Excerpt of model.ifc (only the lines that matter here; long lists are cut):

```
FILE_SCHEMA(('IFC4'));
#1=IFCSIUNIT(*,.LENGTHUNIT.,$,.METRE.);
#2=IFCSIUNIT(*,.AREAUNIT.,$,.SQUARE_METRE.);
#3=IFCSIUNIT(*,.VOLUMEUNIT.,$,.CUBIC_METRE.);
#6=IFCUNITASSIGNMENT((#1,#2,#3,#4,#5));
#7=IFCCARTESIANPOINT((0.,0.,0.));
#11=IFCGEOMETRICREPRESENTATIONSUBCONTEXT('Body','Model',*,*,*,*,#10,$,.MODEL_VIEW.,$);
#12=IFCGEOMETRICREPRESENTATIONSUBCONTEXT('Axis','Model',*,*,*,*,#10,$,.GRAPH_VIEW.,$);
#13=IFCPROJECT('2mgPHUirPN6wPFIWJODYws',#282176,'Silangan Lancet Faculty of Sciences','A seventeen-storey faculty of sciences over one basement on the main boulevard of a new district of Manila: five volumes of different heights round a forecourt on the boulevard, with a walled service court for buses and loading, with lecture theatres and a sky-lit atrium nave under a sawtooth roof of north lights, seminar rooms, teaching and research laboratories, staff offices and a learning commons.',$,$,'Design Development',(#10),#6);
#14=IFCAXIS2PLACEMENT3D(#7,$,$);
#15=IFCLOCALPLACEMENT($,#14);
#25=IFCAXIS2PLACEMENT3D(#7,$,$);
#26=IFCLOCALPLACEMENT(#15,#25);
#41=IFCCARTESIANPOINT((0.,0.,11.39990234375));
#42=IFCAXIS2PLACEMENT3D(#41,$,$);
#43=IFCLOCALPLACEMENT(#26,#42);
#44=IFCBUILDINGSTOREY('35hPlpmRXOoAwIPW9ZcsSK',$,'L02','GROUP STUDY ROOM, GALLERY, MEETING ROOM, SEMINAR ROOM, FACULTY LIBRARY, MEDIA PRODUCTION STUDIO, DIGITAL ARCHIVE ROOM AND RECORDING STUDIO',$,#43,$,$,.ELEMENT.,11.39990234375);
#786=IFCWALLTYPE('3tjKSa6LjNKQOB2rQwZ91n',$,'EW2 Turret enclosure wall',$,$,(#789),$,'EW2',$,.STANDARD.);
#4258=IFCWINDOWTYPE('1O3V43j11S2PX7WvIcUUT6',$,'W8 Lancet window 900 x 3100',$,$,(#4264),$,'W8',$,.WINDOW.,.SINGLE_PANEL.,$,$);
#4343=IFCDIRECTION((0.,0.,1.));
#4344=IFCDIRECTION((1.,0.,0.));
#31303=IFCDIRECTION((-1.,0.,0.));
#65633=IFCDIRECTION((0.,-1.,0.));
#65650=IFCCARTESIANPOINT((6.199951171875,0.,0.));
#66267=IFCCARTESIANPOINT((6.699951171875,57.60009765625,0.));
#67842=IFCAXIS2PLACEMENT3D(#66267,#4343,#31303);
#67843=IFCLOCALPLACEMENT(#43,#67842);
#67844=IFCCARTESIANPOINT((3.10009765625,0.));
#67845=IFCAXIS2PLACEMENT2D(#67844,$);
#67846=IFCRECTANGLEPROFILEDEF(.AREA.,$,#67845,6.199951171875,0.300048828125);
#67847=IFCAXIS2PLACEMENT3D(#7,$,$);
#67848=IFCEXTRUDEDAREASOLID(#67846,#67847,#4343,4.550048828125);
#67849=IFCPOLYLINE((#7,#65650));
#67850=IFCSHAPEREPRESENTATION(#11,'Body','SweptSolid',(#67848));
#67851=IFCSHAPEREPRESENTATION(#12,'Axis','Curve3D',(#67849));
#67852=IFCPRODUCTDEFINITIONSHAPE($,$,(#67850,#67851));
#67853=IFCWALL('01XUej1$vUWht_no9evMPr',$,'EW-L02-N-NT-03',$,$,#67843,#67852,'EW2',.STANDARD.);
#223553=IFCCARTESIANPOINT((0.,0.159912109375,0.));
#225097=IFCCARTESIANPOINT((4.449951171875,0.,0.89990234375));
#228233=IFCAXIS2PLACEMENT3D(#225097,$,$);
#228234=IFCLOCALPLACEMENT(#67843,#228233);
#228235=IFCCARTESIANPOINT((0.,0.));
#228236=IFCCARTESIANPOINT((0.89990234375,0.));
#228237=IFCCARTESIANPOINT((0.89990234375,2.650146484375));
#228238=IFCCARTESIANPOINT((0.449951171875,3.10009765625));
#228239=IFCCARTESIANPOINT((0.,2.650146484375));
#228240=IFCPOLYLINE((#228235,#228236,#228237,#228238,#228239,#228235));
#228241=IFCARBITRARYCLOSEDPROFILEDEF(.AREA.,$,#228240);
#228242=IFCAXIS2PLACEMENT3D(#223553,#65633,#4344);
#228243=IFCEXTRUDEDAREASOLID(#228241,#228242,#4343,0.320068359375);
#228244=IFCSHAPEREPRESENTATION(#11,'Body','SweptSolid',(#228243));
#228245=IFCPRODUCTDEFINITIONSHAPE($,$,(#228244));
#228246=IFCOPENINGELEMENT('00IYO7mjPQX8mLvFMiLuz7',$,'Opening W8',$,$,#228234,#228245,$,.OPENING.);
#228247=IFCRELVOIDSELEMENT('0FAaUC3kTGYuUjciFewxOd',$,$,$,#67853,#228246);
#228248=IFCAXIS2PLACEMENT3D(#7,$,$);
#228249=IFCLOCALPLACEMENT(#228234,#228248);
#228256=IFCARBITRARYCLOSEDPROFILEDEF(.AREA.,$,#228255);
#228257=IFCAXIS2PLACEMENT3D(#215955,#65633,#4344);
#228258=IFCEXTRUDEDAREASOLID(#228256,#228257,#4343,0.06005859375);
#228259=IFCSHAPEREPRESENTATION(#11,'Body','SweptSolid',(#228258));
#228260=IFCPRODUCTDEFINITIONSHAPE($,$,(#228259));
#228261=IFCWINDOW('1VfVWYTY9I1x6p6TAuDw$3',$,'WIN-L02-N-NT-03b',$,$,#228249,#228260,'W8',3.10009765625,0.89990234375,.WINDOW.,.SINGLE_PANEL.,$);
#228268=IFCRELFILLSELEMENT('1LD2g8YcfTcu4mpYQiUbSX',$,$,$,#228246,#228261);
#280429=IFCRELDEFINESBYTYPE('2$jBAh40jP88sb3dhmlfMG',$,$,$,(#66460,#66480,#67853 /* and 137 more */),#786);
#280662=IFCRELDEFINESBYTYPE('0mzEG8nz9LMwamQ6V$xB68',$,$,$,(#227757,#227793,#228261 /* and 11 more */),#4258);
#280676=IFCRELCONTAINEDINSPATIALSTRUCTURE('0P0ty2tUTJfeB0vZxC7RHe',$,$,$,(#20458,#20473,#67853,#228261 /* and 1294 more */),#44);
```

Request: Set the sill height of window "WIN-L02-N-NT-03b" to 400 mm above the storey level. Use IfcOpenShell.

```python
import numpy as np
import ifcopenshell
import ifcopenshell.api.geometry
import ifcopenshell.geom
import ifcopenshell.util.element
import ifcopenshell.util.placement
import ifcopenshell.util.shape
import ifcopenshell.util.unit

model = ifcopenshell.open("model.ifc")
unit_scale = ifcopenshell.util.unit.calculate_unit_scale(model)

window = model.by_guid("1VfVWYTY9I1x6p6TAuDw$3")
opening = window.FillsVoids[0].RelatingOpeningElement
storey = ifcopenshell.util.element.get_container(window, ifc_class="IfcBuildingStorey")
level = ifcopenshell.util.placement.get_local_placement(storey.ObjectPlacement)[2, 3]

# The opening's origin need not be at the sill, so measure its lowest point.
shape = ifcopenshell.geom.create_shape(ifcopenshell.geom.settings(), opening)
bottom = ifcopenshell.util.shape.get_shape_bottom_elevation(shape, shape.geometry) / unit_scale
dz = level + 0.4 - bottom

shift = np.array([0.0, 0.0, dz])
# The window is placed relative to its opening, so it follows when the opening moves.
matrix = ifcopenshell.util.placement.get_local_placement(opening.ObjectPlacement)
matrix[:3, 3] += shift
ifcopenshell.api.geometry.edit_object_placement(
    model, product=opening, matrix=matrix, is_si=False, should_transform_children=True
)

print(f"moved by {dz * unit_scale:+.3f} m")

model.write("model_rev.ifc")
```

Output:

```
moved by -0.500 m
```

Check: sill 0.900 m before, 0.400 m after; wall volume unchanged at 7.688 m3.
